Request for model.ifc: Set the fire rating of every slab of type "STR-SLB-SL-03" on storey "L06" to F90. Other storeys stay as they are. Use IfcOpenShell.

First a look at what the model holds.

```python
import ifcopenshell
import ifcopenshell.util.element

model = ifcopenshell.open("model.ifc")
print(model.schema)
storey = next(s for s in model.by_type("IfcBuildingStorey") if s.Name == "L06")
slabs = [e for e in ifcopenshell.util.element.get_decomposition(storey) if e.is_a("IfcSlab")]
seen = {}
for e in slabs:
    element_type = ifcopenshell.util.element.get_type(e)
    key = (element_type.Name if element_type != e and element_type else None, ifcopenshell.util.element.get_pset(e, "Pset_SlabCommon", "FireRating"))
    seen[key] = seen.get(key, 0) + 1
for (name, value), count in sorted(seen.items(), key=str):
    print(count, "x", name, "|", value)
```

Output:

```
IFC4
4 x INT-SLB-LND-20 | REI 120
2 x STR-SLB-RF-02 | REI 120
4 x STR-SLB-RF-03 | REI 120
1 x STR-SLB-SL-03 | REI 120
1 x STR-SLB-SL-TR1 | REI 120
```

```python
import ifcopenshell
import ifcopenshell.api.pset
import ifcopenshell.util.element

model = ifcopenshell.open("model.ifc")

storey = next(s for s in model.by_type("IfcBuildingStorey") if s.Name == "L06")
slabs = [e for e in ifcopenshell.util.element.get_decomposition(storey) if e.is_a("IfcSlab")]

count = 0
for e in slabs:
    element_type = ifcopenshell.util.element.get_type(e)
    if element_type in (None, e) or element_type.Name != "STR-SLB-SL-03":
        continue
    # add_pset returns the element's existing set when there is one.
    pset = ifcopenshell.api.pset.add_pset(model, product=e, name="Pset_SlabCommon")
    ifcopenshell.api.pset.edit_pset(model, pset=pset, properties={"FireRating": "F90"})
    count += 1

print(count, "slabs updated")

model.write("model_rev.ifc")
```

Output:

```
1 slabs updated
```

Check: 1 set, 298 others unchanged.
